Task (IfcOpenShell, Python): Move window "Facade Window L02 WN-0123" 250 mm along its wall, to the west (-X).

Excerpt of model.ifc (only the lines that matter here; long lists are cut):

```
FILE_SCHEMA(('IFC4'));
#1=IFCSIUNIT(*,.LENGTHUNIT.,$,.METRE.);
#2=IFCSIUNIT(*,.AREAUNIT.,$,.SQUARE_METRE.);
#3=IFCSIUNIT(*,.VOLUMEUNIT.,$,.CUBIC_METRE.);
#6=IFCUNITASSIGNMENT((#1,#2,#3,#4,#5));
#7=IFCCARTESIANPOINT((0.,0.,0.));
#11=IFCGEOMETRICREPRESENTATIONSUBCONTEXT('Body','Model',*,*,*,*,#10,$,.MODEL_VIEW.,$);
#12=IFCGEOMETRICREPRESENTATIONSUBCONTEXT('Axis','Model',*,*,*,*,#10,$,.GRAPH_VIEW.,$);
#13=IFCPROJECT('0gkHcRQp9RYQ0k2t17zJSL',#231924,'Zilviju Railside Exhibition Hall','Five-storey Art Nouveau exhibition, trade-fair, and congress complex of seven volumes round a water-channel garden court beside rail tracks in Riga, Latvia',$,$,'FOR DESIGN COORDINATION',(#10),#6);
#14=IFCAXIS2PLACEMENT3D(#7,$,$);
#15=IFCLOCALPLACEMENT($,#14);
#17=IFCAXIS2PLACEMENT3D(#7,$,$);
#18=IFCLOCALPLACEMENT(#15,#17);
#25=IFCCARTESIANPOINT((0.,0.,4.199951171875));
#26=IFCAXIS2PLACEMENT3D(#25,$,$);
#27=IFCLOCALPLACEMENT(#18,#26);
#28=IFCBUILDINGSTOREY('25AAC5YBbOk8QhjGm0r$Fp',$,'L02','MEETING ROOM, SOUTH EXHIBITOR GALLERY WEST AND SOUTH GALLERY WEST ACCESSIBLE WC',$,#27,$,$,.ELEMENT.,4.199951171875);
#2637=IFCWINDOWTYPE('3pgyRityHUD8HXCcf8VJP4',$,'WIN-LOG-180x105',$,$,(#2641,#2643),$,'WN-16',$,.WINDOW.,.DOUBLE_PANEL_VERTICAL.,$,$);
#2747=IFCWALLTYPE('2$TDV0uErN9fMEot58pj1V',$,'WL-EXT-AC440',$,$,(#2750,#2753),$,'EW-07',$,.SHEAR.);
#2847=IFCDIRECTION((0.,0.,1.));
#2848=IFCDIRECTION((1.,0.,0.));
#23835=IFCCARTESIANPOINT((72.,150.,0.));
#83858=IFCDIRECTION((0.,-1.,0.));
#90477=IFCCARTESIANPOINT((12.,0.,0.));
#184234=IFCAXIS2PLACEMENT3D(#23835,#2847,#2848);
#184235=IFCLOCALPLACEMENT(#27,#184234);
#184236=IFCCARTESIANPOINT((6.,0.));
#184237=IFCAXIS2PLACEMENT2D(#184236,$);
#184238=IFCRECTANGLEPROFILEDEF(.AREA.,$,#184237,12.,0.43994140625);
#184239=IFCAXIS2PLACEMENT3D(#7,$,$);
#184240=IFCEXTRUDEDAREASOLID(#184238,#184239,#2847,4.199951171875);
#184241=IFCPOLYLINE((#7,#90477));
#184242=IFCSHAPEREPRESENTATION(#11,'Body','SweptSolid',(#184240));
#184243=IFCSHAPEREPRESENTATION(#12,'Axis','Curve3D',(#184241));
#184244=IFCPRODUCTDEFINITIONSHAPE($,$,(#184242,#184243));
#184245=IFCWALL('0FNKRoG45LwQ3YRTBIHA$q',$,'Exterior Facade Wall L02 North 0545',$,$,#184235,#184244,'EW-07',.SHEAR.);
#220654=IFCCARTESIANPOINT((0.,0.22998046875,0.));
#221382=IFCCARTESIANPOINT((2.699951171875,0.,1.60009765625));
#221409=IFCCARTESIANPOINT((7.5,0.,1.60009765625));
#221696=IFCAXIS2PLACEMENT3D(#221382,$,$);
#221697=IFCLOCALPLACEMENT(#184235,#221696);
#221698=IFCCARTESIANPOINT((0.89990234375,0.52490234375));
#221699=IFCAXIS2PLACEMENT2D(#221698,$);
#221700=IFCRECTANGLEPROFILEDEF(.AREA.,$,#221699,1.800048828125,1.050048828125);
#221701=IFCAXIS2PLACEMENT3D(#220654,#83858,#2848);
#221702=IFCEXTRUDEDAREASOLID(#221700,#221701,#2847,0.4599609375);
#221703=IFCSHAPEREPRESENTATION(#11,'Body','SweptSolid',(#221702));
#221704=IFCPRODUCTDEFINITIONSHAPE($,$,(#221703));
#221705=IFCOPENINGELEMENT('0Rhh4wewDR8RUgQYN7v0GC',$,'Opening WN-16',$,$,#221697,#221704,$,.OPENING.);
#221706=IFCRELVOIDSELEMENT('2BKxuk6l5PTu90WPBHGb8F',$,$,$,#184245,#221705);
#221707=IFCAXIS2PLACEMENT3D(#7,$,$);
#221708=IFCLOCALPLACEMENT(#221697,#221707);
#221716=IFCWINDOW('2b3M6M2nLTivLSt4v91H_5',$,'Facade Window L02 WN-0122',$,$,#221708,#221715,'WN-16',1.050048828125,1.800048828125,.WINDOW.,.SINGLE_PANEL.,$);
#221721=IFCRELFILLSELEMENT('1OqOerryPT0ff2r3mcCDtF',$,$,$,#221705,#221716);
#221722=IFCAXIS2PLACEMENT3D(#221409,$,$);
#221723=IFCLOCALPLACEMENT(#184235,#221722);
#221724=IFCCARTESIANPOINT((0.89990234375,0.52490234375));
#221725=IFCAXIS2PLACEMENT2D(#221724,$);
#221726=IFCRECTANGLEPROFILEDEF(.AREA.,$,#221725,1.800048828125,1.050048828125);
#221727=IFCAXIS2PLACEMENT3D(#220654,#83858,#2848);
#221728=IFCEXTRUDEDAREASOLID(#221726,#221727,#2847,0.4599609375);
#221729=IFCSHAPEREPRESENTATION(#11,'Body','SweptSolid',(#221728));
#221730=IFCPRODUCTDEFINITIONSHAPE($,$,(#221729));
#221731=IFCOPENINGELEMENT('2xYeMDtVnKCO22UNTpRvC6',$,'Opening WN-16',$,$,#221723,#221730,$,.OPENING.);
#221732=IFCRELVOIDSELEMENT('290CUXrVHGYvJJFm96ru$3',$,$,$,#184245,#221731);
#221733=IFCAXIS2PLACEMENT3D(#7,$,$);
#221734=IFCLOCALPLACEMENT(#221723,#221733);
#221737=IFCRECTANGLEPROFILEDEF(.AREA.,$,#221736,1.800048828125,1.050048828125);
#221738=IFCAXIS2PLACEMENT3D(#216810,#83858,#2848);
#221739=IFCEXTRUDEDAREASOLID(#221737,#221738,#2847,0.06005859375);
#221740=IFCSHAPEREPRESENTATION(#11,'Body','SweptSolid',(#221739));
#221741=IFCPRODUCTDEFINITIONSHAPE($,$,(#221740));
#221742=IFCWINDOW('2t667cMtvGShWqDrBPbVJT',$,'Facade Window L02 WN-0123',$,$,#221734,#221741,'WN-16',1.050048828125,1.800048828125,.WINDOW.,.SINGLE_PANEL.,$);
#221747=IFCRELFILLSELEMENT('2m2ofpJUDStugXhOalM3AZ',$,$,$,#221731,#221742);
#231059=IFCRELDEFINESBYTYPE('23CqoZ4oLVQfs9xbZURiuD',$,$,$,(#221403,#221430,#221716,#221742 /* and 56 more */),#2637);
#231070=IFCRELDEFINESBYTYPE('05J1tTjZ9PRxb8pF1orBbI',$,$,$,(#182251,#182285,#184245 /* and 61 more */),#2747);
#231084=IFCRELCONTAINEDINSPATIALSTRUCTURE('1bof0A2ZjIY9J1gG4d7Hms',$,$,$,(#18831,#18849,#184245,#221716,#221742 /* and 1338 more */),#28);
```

```python
import ifcopenshell
import ifcopenshell.api.geometry
import ifcopenshell.util.placement

model = ifcopenshell.open("model.ifc")

window = model.by_id(221742)
opening = window.FillsVoids[0].RelatingOpeningElement
wall = opening.VoidsElements[0].RelatingBuildingElement

wall_matrix = ifcopenshell.util.placement.get_local_placement(wall.ObjectPlacement)
shift = wall_matrix[:3, 0] * -0.25
before = ifcopenshell.util.placement.get_local_placement(window.ObjectPlacement)[:3, 3].copy()

# The window is placed relative to its opening, so it follows when the opening moves.
matrix = ifcopenshell.util.placement.get_local_placement(opening.ObjectPlacement)
matrix[:3, 3] += shift
ifcopenshell.api.geometry.edit_object_placement(
    model, product=opening, matrix=matrix, is_si=False, should_transform_children=True
)

after = ifcopenshell.util.placement.get_local_placement(window.ObjectPlacement)[:3, 3]
print("window moved by", (after - before).round(3) + 0.0)

model.write("model_v2.ifc")
```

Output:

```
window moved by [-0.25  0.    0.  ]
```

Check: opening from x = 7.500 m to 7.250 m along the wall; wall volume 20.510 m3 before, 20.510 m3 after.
